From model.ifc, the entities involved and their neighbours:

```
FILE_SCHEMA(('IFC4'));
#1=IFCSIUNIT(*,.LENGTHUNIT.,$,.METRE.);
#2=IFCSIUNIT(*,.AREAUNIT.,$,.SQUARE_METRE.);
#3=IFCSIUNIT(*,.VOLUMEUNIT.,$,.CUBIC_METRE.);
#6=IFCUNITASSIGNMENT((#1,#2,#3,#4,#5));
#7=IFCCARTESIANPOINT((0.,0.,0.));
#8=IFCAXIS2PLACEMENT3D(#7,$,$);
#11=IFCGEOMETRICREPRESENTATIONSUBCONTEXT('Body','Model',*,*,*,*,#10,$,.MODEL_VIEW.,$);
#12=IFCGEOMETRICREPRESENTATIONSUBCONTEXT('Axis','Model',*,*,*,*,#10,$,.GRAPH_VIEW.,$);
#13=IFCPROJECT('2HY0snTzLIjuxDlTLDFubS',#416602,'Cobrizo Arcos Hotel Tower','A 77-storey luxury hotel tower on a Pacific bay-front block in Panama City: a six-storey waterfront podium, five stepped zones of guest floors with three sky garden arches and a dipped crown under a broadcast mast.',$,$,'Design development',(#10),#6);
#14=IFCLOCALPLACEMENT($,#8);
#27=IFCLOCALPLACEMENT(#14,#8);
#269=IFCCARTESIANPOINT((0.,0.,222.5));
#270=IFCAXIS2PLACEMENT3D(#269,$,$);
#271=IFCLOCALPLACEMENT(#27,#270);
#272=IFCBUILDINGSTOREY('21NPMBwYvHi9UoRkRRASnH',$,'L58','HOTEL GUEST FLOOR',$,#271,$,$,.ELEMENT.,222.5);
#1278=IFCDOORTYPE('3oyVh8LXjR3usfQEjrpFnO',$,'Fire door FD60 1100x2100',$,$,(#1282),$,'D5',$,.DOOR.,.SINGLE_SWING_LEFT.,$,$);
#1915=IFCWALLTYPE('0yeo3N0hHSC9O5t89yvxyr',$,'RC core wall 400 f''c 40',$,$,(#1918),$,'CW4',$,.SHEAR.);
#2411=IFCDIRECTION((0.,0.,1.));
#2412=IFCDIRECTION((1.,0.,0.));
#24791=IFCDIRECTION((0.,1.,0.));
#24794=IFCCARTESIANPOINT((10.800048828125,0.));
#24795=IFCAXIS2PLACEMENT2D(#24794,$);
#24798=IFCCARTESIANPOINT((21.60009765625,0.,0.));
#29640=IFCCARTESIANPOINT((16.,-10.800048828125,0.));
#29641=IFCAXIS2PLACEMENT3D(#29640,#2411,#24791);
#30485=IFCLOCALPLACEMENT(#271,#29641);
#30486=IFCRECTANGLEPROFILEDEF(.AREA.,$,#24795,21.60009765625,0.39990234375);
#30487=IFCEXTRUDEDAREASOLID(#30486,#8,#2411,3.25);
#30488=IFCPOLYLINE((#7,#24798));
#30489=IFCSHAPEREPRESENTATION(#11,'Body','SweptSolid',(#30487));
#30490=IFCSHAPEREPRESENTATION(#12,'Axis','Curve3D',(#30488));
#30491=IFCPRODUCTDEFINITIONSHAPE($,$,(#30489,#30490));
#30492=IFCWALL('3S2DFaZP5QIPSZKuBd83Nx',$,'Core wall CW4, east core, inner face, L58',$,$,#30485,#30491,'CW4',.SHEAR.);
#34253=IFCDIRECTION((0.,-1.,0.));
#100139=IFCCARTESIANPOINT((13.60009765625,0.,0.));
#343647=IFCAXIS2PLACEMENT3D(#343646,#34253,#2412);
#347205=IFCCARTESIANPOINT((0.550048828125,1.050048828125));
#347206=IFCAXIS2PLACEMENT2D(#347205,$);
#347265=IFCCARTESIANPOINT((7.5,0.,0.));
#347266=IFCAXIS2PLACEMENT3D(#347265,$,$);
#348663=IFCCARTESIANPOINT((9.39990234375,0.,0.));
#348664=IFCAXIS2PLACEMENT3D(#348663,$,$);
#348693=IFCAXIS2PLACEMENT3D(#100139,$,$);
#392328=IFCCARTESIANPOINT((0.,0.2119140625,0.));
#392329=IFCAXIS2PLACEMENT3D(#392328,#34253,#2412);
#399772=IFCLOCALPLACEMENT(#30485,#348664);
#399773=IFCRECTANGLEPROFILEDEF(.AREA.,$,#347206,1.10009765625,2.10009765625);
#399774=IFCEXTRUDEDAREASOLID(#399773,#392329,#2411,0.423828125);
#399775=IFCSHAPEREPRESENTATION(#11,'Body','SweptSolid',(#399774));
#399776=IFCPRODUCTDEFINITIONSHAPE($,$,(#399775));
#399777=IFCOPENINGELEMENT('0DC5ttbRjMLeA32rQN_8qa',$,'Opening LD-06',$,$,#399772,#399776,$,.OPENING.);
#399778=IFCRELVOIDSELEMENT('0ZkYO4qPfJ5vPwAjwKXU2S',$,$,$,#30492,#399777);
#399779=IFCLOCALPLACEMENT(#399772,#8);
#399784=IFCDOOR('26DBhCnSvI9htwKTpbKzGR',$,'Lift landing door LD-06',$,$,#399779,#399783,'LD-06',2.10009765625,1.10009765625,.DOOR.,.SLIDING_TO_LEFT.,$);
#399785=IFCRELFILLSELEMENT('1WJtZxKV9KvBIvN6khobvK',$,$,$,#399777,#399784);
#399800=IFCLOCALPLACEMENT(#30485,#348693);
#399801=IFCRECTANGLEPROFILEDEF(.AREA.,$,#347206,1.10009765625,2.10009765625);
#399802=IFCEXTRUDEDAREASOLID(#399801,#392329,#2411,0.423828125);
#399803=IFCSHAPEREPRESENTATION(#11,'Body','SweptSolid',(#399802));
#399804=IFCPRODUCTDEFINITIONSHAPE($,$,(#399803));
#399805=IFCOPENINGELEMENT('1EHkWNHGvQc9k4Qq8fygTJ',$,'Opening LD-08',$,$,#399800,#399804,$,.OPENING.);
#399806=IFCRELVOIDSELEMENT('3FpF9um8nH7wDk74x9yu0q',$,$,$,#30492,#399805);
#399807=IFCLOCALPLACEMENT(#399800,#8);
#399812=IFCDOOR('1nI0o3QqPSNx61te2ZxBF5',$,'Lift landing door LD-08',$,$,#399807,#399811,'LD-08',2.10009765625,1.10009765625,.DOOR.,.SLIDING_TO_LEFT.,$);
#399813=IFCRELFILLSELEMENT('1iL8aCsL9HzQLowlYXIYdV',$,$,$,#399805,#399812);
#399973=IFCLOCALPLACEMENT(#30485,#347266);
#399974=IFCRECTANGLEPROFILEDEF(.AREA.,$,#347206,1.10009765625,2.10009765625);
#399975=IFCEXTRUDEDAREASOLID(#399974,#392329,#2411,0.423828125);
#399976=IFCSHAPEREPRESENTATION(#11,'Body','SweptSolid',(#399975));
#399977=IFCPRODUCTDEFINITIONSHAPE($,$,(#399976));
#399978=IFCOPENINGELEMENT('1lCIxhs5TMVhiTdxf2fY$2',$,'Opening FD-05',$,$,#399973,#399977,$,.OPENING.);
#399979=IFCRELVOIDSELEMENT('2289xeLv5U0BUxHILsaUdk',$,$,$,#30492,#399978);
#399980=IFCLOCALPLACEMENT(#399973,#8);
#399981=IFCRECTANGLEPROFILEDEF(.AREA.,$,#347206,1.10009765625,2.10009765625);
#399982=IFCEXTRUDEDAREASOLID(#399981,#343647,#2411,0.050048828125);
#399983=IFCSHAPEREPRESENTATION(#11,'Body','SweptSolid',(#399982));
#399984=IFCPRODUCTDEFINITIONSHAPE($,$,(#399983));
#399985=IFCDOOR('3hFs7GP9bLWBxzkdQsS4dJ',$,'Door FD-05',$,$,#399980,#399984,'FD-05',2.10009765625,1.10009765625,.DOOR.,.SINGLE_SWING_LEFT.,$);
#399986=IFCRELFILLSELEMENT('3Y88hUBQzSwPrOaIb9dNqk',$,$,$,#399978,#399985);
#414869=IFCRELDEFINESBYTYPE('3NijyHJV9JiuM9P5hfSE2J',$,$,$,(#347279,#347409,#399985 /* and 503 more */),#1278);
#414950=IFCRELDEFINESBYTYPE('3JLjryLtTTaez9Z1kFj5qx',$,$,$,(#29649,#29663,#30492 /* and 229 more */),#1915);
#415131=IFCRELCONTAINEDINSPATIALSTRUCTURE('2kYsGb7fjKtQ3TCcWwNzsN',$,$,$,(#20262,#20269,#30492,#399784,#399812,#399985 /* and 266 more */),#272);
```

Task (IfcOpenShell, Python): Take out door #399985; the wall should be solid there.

```python
import ifcopenshell
import ifcopenshell.api.feature
import ifcopenshell.api.root
import ifcopenshell.geom
import ifcopenshell.util.shape

model = ifcopenshell.open("model.ifc")
settings = ifcopenshell.geom.settings()


def volume(element):
    """Net volume in cubic metres, openings subtracted."""
    shape = ifcopenshell.geom.create_shape(settings, element)
    return ifcopenshell.util.shape.get_volume(shape.geometry)


door = model.by_guid("3hFs7GP9bLWBxzkdQsS4dJ")
opening = door.FillsVoids[0].RelatingOpeningElement
wall = opening.VoidsElements[0].RelatingBuildingElement
before = volume(wall)

ifcopenshell.api.root.remove_product(model, product=door)
ifcopenshell.api.feature.remove_feature(model, feature=opening)

after = volume(wall)

print(f"wall volume {before:.3f} -> {after:.3f} m3")

model.write("model_edited.ifc")
```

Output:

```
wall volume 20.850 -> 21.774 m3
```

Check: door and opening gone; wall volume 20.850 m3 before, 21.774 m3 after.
